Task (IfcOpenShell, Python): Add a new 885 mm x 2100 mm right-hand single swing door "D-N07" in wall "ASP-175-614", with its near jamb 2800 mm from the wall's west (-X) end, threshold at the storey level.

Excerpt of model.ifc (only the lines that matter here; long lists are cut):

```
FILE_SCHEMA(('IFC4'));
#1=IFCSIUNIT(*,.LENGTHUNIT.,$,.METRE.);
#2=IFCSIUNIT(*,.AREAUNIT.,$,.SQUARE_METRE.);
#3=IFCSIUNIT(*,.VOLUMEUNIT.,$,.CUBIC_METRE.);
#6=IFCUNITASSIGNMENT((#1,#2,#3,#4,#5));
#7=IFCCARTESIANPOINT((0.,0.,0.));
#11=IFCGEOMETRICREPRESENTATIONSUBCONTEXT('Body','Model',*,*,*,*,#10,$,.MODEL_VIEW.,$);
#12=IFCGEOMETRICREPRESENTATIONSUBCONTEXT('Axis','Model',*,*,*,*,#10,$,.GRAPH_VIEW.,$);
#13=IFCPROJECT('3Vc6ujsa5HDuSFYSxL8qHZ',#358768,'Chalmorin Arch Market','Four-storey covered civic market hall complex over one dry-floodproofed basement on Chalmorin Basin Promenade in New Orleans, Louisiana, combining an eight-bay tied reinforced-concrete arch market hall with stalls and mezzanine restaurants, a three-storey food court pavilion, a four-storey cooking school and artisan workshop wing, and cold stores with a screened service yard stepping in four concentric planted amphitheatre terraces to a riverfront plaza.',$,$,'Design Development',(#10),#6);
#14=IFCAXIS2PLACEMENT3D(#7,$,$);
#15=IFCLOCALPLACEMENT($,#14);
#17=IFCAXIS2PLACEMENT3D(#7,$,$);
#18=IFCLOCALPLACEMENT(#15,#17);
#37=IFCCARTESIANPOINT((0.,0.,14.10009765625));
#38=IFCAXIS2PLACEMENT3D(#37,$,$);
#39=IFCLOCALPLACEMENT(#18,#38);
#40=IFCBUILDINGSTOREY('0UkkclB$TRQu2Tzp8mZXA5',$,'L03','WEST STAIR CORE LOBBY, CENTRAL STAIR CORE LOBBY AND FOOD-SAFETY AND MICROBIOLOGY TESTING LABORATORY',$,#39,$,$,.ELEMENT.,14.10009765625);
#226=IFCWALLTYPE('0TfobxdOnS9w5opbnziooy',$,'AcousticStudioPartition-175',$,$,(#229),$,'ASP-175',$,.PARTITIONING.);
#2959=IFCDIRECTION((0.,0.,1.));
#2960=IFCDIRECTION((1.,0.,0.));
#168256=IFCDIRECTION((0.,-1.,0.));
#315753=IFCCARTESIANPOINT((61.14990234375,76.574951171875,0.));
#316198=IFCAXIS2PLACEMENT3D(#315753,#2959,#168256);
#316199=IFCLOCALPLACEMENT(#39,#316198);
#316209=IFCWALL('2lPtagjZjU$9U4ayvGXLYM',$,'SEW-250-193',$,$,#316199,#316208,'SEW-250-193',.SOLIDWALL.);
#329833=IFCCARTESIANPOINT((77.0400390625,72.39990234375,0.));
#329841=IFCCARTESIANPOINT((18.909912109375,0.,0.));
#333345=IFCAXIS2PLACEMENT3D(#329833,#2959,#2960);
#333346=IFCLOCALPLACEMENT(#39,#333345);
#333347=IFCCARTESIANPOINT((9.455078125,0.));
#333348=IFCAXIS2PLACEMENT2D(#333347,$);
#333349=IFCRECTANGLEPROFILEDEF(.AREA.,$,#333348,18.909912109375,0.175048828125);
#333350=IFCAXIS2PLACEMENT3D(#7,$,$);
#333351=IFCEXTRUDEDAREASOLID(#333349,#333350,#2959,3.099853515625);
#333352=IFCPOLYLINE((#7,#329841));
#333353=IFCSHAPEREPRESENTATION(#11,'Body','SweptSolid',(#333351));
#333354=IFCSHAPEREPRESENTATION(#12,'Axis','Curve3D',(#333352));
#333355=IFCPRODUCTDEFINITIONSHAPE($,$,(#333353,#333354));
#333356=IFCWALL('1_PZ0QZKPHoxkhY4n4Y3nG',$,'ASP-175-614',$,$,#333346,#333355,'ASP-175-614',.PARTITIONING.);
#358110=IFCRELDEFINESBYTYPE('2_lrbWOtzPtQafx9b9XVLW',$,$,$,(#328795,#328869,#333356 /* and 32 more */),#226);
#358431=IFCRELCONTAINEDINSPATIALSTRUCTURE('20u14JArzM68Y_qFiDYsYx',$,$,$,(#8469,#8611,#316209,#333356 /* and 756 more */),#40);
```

```python
import numpy as np
import ifcopenshell
import ifcopenshell.api.feature
import ifcopenshell.api.geometry
import ifcopenshell.api.root
import ifcopenshell.api.spatial
import ifcopenshell.geom
import ifcopenshell.util.element
import ifcopenshell.util.placement
import ifcopenshell.util.representation
import ifcopenshell.util.shape
import ifcopenshell.util.unit

model = ifcopenshell.open("model.ifc")
unit_scale = ifcopenshell.util.unit.calculate_unit_scale(model)
settings = ifcopenshell.geom.settings()


def volume(element):
    """Net volume in cubic metres, openings subtracted."""
    shape = ifcopenshell.geom.create_shape(settings, element)
    return ifcopenshell.util.shape.get_volume(shape.geometry)


wall = model.by_guid("1_PZ0QZKPHoxkhY4n4Y3nG")
storey = ifcopenshell.util.element.get_container(wall, ifc_class="IfcBuildingStorey")
context = ifcopenshell.util.representation.get_context(model, "Model", "Body", "MODEL_VIEW")
before = volume(wall)

width, height, from_end, sill = 0.885, 2.1, 2.8, 0.0  # metres

# The wall runs along its own X axis, and the end named is its -X end.
wall_shape = ifcopenshell.geom.create_shape(settings, wall)
x, y, z = ifcopenshell.util.shape.get_vertices(wall_shape.geometry).T
start = x.min() + from_end
face, thickness = float(y.min()), float(y.max() - y.min())
wall_matrix = ifcopenshell.util.placement.get_local_placement(wall.ObjectPlacement)
level = ifcopenshell.util.placement.get_local_placement(storey.ObjectPlacement)[2, 3]


def in_wall(x, y):
    """Placement at x, y metres in the wall's axes, at sill height."""
    matrix = wall_matrix.copy()
    matrix[:, 3] = wall_matrix @ np.array([x / unit_scale, y / unit_scale, 0.0, 1.0])
    matrix[2, 3] = level + sill / unit_scale
    return matrix


# Opening: a box that overshoots both wall faces by 50 mm.
opening = ifcopenshell.api.root.create_entity(model, ifc_class="IfcOpeningElement", predefined_type="OPENING")
box = ifcopenshell.api.geometry.add_wall_representation(
    model, context=context, length=width, height=height, thickness=thickness + 0.1
)
ifcopenshell.api.geometry.assign_representation(model, product=opening, representation=box)
ifcopenshell.api.geometry.edit_object_placement(model, product=opening, matrix=in_wall(start, face - 0.05), is_si=False)
ifcopenshell.api.feature.add_feature(model, feature=opening, element=wall)

door = ifcopenshell.api.root.create_entity(model, ifc_class="IfcDoor", name="D-N07", predefined_type="DOOR")
door.OverallWidth, door.OverallHeight = width / unit_scale, height / unit_scale
door.OperationType = "SINGLE_SWING_RIGHT"
body = ifcopenshell.api.geometry.add_door_representation(
    model,
    context=context,
    overall_width=door.OverallWidth,
    overall_height=door.OverallHeight,
    operation_type="SINGLE_SWING_RIGHT",
    lining_properties={"LiningDepth": thickness / unit_scale, "ThresholdDepth": thickness / unit_scale},
)
ifcopenshell.api.geometry.assign_representation(model, product=door, representation=body)
ifcopenshell.api.spatial.assign_container(model, products=[door], relating_structure=storey)
ifcopenshell.api.feature.add_filling(model, opening=opening, element=door)

# The lining spans the wall, so the door starts at the wall face.
ifcopenshell.api.geometry.edit_object_placement(model, product=door, matrix=in_wall(start, face), is_si=False)

after = volume(wall)

print(f"wall volume {before:.3f} -> {after:.3f} m3")

model.write("model_edited.ifc")
```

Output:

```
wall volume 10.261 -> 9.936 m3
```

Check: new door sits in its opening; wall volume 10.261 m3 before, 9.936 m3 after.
